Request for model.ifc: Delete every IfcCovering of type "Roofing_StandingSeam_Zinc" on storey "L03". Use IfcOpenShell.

First a look at what the model holds.

```python
import ifcopenshell
import ifcopenshell.util.element

model = ifcopenshell.open("model.ifc")
print(model.schema)
storey = next(s for s in model.by_type("IfcBuildingStorey") if s.Name == "L03")
coverings = [e for e in ifcopenshell.util.element.get_decomposition(storey) if e.is_a("IfcCovering")]
seen = {}
for e in coverings:
    element_type = ifcopenshell.util.element.get_type(e)
    name = element_type.Name if element_type not in (None, e) else None
    seen[name] = seen.get(name, 0) + 1
for name, count in sorted(seen.items(), key=str):
    print(count, "x", name)
```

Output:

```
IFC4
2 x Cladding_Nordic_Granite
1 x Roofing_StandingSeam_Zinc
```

```python
import ifcopenshell
import ifcopenshell.api.root
import ifcopenshell.util.element

model = ifcopenshell.open("model.ifc")

storey = next(s for s in model.by_type("IfcBuildingStorey") if s.Name == "L03")
coverings = [e for e in ifcopenshell.util.element.get_decomposition(storey) if e.is_a("IfcCovering")]
targets = [e for e in coverings if (t := ifcopenshell.util.element.get_type(e)) not in (None, e) and t.Name == "Roofing_StandingSeam_Zinc"]

for e in targets:
    ifcopenshell.api.root.remove_product(model, product=e)
print(len(targets), "removed")

model.write("model_v2.ifc")
```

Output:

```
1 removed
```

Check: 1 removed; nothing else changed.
